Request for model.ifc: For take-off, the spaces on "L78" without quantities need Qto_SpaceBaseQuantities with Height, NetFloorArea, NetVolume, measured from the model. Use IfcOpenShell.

First a look at what the model holds.

```python
import ifcopenshell
import ifcopenshell.util.element
import ifcopenshell.util.unit

model = ifcopenshell.open("model.ifc")
print(model.schema)
for unit_type in ("LENGTHUNIT", "AREAUNIT", "VOLUMEUNIT"):
    print(unit_type, ifcopenshell.util.unit.calculate_unit_scale(model, unit_type))
storey = next(s for s in model.by_type("IfcBuildingStorey") if s.Name == "L78")
spaces = [e for e in ifcopenshell.util.element.get_decomposition(storey) if e.is_a("IfcSpace")]
for e in sorted(spaces, key=lambda e: e.id()):
    print(e.id(), e.is_a(), e.Name, list(ifcopenshell.util.element.get_psets(e, qtos_only=True)), sep=" | ")
```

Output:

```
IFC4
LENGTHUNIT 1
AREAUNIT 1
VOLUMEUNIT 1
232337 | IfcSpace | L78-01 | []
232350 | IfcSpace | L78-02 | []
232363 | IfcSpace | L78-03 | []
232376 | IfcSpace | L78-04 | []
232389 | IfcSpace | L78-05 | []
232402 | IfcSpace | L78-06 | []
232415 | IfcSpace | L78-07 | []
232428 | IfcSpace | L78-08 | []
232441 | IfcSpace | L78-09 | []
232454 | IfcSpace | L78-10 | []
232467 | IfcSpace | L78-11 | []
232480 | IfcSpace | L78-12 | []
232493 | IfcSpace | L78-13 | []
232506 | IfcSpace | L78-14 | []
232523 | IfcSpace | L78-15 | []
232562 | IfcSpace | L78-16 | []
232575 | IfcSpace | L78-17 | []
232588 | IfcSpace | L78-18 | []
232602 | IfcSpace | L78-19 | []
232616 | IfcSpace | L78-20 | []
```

```python
import ifcopenshell
import ifcopenshell.api.pset
import ifcopenshell.geom
import ifcopenshell.util.element
import ifcopenshell.util.shape
import ifcopenshell.util.unit

model = ifcopenshell.open("model.ifc")
unit_scale = ifcopenshell.util.unit.calculate_unit_scale(model)
area_scale = ifcopenshell.util.unit.calculate_unit_scale(model, "AREAUNIT")
volume_scale = ifcopenshell.util.unit.calculate_unit_scale(model, "VOLUMEUNIT")
settings = ifcopenshell.geom.settings()

storey = next(s for s in model.by_type("IfcBuildingStorey") if s.Name == "L78")
spaces = [e for e in ifcopenshell.util.element.get_decomposition(storey) if e.is_a("IfcSpace")]

for e in sorted(spaces, key=lambda e: e.id()):
    if ifcopenshell.util.element.get_psets(e, qtos_only=True, should_inherit=False):
        continue
    # Geometry comes back in metres, in the element's own axes.
    shape = ifcopenshell.geom.create_shape(settings, e)
    values = {
        "Height": ifcopenshell.util.shape.get_z(shape.geometry) / unit_scale,
        "NetFloorArea": ifcopenshell.util.shape.get_footprint_area(shape.geometry) / area_scale,
        "NetVolume": ifcopenshell.util.shape.get_volume(shape.geometry) / volume_scale,
    }
    qto = ifcopenshell.api.pset.add_qto(model, product=e, name="Qto_SpaceBaseQuantities")
    ifcopenshell.api.pset.edit_qto(model, qto=qto, properties=values)
    print(e.id(), {k: round(v, 3) for k, v in values.items()})

model.write("model_edited.ifc")
```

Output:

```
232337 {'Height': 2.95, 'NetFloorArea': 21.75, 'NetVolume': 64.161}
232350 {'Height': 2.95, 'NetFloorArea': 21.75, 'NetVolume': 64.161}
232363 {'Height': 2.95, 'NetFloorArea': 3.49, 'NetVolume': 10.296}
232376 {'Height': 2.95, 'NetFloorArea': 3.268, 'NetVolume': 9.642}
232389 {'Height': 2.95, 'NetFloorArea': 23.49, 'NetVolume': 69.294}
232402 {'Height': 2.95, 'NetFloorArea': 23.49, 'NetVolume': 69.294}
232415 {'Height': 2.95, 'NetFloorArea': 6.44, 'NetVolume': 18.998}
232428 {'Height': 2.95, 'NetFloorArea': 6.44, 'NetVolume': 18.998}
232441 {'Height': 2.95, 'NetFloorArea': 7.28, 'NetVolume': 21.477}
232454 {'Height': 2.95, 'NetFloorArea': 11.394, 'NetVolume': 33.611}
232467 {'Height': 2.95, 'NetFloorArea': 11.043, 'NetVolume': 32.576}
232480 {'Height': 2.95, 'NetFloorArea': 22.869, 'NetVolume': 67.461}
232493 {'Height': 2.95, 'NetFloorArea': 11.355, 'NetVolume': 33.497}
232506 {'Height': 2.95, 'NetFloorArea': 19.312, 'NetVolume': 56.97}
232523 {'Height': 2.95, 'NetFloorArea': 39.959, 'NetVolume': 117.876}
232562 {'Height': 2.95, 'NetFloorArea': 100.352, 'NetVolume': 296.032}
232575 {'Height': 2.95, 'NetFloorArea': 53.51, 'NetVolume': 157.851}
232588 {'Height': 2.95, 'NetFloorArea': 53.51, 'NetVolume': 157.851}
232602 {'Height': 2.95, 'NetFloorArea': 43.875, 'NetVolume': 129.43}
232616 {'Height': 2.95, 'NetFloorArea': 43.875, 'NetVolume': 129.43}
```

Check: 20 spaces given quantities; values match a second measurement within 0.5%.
